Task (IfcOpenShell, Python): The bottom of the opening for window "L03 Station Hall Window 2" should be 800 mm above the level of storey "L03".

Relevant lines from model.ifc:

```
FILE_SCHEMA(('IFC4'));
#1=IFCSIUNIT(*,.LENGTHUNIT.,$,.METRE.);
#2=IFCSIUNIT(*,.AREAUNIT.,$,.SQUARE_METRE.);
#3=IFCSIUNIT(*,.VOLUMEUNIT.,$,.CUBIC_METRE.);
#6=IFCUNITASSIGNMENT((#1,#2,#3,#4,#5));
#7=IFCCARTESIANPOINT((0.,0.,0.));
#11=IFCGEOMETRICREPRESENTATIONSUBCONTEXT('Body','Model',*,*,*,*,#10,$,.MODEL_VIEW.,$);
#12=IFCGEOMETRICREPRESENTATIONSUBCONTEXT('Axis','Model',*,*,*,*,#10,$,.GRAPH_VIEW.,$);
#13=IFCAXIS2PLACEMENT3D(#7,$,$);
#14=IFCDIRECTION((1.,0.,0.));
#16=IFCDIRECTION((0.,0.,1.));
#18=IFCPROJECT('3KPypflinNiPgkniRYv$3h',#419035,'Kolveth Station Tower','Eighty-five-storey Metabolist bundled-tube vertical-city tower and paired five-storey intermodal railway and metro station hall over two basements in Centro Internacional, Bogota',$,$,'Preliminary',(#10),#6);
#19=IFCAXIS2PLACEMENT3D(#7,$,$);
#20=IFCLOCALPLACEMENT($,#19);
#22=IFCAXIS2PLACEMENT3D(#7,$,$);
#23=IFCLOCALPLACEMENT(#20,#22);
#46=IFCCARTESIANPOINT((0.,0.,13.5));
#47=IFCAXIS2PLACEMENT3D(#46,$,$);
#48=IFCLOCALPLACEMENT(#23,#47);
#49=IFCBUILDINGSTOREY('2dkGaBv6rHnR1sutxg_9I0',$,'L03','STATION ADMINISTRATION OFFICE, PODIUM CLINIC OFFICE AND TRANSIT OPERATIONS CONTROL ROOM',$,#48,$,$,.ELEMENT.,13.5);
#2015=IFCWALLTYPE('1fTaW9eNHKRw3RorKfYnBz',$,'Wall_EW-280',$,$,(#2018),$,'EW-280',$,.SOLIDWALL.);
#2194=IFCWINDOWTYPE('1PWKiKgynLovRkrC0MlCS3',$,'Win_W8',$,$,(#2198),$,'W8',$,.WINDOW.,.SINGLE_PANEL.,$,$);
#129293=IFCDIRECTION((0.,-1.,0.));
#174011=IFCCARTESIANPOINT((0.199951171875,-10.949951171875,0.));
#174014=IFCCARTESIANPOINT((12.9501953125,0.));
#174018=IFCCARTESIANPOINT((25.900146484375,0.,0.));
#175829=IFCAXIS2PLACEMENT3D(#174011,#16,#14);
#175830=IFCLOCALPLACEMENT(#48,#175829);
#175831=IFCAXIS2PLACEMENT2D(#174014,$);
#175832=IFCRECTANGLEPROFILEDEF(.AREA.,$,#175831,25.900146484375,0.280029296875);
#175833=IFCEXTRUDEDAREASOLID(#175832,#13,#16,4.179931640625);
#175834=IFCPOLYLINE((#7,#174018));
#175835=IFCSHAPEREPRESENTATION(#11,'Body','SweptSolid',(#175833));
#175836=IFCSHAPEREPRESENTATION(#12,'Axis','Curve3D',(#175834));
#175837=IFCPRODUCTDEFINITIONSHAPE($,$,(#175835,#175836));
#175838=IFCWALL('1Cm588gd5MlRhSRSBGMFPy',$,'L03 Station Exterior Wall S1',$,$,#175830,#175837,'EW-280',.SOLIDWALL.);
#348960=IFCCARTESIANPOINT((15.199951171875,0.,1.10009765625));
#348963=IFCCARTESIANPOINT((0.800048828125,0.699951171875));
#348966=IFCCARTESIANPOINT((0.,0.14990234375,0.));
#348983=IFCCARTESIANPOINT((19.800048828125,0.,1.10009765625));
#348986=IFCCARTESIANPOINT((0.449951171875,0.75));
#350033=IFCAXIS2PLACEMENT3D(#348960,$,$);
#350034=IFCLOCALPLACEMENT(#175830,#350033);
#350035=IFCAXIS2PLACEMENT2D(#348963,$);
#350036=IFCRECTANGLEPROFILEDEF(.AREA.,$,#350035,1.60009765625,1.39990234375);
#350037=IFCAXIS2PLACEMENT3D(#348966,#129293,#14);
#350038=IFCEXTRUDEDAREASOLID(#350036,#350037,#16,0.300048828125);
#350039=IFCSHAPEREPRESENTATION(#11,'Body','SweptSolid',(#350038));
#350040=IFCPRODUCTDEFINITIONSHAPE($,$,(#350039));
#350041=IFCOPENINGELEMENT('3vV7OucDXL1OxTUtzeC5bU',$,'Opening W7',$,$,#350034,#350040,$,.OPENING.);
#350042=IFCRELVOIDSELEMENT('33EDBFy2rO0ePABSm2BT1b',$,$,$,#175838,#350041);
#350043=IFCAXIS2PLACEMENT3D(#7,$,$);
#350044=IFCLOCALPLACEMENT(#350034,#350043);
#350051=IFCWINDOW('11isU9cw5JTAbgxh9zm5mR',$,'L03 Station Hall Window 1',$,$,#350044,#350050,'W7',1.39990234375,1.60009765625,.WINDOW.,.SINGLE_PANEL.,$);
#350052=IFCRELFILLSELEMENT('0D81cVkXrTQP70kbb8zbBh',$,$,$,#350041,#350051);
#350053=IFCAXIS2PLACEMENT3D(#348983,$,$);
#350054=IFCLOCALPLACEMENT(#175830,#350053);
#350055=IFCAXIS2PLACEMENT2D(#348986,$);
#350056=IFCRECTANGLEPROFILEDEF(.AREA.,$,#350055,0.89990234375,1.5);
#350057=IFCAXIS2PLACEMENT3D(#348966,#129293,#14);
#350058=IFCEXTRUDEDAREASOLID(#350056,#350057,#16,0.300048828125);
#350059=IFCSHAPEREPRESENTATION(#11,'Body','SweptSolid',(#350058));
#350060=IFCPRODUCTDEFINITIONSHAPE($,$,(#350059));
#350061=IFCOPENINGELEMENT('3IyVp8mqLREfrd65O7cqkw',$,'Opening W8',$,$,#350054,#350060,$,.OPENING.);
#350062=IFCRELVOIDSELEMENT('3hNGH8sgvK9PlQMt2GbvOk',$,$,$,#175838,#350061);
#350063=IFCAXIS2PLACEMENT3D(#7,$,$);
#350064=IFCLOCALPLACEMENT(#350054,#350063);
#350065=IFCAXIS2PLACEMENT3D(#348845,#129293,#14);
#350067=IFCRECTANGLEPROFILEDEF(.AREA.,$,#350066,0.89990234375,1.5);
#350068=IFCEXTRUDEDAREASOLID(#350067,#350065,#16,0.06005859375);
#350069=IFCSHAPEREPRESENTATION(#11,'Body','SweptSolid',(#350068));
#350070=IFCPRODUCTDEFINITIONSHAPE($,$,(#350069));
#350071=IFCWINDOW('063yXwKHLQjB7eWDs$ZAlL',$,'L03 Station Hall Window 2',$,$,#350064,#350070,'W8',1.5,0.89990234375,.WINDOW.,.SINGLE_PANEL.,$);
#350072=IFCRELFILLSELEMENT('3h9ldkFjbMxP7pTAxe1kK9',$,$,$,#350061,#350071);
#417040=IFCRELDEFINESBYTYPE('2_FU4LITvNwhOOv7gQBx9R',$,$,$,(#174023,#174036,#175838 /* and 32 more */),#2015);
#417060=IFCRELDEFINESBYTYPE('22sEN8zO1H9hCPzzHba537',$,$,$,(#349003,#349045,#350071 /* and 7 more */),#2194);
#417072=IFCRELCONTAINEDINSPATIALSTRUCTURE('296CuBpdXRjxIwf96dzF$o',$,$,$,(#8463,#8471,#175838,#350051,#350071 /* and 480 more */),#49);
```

```python
import numpy as np
import ifcopenshell
import ifcopenshell.api.geometry
import ifcopenshell.geom
import ifcopenshell.util.element
import ifcopenshell.util.placement
import ifcopenshell.util.shape
import ifcopenshell.util.unit

model = ifcopenshell.open("model.ifc")
unit_scale = ifcopenshell.util.unit.calculate_unit_scale(model)

window = model.by_id(350071)
opening = window.FillsVoids[0].RelatingOpeningElement
storey = ifcopenshell.util.element.get_container(window, ifc_class="IfcBuildingStorey")
level = ifcopenshell.util.placement.get_local_placement(storey.ObjectPlacement)[2, 3]

# The opening's origin need not be at the sill, so measure its lowest point.
shape = ifcopenshell.geom.create_shape(ifcopenshell.geom.settings(), opening)
bottom = ifcopenshell.util.shape.get_shape_bottom_elevation(shape, shape.geometry) / unit_scale
dz = level + 0.8 / unit_scale - bottom

shift = np.array([0.0, 0.0, dz])
# The window is placed relative to its opening, so it follows when the opening moves.
matrix = ifcopenshell.util.placement.get_local_placement(opening.ObjectPlacement)
matrix[:3, 3] += shift
ifcopenshell.api.geometry.edit_object_placement(
    model, product=opening, matrix=matrix, is_si=False, should_transform_children=True
)

print(f"moved by {dz * unit_scale:+.3f} m")

model.write("model_rev.ifc")
```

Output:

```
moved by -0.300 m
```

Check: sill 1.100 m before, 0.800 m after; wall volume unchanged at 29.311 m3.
